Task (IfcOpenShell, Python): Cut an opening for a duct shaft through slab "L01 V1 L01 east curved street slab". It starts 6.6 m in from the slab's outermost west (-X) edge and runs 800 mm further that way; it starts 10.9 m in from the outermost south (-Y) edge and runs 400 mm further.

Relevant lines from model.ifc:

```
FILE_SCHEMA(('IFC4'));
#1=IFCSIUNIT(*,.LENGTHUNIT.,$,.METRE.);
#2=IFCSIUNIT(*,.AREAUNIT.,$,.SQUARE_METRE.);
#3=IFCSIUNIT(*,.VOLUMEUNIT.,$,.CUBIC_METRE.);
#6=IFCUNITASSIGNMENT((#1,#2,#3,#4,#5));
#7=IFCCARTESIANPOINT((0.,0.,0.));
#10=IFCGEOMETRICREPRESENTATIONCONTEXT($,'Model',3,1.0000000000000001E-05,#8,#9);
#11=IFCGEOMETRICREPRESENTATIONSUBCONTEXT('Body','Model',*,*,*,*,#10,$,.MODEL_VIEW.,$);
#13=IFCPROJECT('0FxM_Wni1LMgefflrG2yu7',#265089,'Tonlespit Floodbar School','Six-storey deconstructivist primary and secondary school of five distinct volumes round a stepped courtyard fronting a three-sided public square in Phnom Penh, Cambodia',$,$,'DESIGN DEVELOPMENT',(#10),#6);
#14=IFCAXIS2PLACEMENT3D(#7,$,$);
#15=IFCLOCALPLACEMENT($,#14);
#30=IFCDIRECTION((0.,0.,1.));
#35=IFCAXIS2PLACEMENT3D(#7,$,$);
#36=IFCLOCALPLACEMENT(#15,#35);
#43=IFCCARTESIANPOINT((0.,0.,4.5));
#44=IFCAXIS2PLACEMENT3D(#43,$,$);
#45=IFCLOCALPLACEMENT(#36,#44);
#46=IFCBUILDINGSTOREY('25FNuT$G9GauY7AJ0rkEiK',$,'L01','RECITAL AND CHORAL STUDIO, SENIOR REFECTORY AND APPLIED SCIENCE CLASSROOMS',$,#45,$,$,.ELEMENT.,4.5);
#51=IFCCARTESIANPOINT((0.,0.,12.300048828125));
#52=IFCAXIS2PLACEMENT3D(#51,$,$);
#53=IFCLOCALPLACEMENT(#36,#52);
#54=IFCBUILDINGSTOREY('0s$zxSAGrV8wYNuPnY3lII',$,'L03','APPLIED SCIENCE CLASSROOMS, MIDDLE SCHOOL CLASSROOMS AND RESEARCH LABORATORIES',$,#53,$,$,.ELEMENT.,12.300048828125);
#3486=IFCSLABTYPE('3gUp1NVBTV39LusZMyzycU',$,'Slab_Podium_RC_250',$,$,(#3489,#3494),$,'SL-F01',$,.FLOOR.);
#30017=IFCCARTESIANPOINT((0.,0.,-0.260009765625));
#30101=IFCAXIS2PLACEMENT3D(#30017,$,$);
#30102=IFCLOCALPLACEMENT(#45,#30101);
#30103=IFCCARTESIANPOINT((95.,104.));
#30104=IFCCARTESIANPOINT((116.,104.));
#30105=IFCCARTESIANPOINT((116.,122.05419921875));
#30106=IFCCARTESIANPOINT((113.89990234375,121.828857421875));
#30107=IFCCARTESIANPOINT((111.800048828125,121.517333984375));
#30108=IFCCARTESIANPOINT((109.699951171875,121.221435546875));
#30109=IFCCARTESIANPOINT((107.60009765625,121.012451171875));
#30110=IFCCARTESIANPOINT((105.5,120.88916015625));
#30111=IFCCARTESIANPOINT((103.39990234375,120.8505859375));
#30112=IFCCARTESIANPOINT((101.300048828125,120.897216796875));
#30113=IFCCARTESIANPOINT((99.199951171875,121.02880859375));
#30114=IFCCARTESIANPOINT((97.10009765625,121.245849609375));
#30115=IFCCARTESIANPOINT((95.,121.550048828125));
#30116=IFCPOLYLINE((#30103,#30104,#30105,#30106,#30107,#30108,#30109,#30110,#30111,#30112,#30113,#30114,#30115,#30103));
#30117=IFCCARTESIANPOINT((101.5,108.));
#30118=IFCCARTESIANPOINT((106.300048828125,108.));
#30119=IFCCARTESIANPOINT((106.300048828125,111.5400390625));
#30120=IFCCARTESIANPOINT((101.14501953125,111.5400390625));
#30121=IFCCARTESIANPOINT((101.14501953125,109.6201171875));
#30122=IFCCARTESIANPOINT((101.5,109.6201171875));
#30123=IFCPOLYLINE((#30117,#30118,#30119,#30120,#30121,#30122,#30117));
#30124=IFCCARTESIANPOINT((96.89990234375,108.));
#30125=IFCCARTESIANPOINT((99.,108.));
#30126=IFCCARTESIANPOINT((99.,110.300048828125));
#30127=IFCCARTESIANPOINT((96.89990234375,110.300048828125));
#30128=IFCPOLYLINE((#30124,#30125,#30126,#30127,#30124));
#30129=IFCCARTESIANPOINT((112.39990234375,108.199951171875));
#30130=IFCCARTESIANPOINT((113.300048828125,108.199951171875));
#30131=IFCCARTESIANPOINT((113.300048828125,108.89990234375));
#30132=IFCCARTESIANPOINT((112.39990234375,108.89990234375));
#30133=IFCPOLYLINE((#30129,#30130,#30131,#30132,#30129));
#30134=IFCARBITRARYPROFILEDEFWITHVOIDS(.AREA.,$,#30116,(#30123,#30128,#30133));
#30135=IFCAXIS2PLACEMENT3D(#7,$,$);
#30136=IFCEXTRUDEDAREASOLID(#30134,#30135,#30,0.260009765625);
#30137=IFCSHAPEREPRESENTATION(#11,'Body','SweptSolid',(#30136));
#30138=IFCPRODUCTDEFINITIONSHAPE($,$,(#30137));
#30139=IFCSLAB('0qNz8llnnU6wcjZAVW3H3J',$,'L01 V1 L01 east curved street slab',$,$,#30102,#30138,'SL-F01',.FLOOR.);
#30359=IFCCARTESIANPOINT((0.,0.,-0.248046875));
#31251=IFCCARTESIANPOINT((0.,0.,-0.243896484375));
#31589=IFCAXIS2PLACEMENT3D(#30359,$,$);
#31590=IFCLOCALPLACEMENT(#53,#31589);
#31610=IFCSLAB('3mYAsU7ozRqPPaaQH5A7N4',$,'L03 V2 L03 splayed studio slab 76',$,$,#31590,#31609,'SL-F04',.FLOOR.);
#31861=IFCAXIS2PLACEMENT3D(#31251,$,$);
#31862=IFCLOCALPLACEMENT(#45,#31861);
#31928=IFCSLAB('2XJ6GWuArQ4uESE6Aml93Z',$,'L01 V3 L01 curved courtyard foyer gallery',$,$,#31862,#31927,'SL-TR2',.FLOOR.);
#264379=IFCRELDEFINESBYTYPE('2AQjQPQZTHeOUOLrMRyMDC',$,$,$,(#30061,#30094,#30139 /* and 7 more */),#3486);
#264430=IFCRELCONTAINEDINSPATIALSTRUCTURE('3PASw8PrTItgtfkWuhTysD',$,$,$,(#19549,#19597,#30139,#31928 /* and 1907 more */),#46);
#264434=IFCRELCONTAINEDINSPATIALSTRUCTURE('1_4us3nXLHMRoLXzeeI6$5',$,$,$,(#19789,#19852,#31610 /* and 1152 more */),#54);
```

```python
import numpy as np
import ifcopenshell
import ifcopenshell.api.feature
import ifcopenshell.api.geometry
import ifcopenshell.api.root
import ifcopenshell.geom
import ifcopenshell.util.placement
import ifcopenshell.util.representation
import ifcopenshell.util.shape
import ifcopenshell.util.unit

model = ifcopenshell.open("model.ifc")
unit_scale = ifcopenshell.util.unit.calculate_unit_scale(model)
settings = ifcopenshell.geom.settings()


def volume(element):
    """Net volume in cubic metres, openings subtracted."""
    shape = ifcopenshell.geom.create_shape(settings, element)
    return ifcopenshell.util.shape.get_volume(shape.geometry)


slab = model.by_id(30139)
before = volume(slab)

# Extent in the slab's own axes, in metres. The edges named are its -X and -Y sides.
slab_shape = ifcopenshell.geom.create_shape(settings, slab)
vertices = ifcopenshell.util.shape.get_vertices(slab_shape.geometry)
x_min, y_min, bottom = vertices.min(axis=0)
top = vertices[:, 2].max()

opening = ifcopenshell.api.root.create_entity(model, ifc_class="IfcOpeningElement", name="Duct shaft opening", predefined_type="OPENING")
context = ifcopenshell.util.representation.get_context(model, "Model", "Body", "MODEL_VIEW")
width, depth = 0.8, 0.4
outline = [(0.0, 0.0), (width, 0.0), (width, depth), (0.0, depth), (0.0, 0.0)]
# Overshoot both faces by 50 mm so the cut is clean.
shape = ifcopenshell.api.geometry.add_slab_representation(
    model, context=context, depth=top - bottom + 0.1, polyline=outline
)
ifcopenshell.api.geometry.assign_representation(model, product=opening, representation=shape)

matrix = ifcopenshell.util.placement.get_local_placement(slab.ObjectPlacement)
matrix[:, 3] = matrix @ np.append(np.array([x_min + 6.6, y_min + 10.9, bottom - 0.05]) / unit_scale, 1.0)
ifcopenshell.api.geometry.edit_object_placement(model, product=opening, matrix=matrix, is_si=False)
ifcopenshell.api.feature.add_feature(model, feature=opening, element=slab)

after = volume(slab)

print(f"slab volume {before:.3f} -> {after:.3f} m3")

model.write("model_updated.ifc")
```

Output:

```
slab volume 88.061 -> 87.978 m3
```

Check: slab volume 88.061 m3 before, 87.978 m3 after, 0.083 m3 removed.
